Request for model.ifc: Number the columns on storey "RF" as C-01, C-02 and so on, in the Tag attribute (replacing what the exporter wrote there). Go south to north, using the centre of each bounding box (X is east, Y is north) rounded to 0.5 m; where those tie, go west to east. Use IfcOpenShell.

First a look at what the model holds.

```python
import ifcopenshell
import ifcopenshell.util.element
import ifcopenshell.util.placement

model = ifcopenshell.open("model.ifc")
print(model.schema)
storey = next(s for s in model.by_type("IfcBuildingStorey") if s.Name == "RF")
columns = [e for e in ifcopenshell.util.element.get_decomposition(storey) if e.is_a("IfcColumn")]
for e in sorted(columns, key=lambda e: e.id()):
    origin = ifcopenshell.util.placement.get_local_placement(e.ObjectPlacement)[:3, 3]
    print(e.id(), e.Tag, e.Name, origin.round(2) + 0.0, sep=" | ")
```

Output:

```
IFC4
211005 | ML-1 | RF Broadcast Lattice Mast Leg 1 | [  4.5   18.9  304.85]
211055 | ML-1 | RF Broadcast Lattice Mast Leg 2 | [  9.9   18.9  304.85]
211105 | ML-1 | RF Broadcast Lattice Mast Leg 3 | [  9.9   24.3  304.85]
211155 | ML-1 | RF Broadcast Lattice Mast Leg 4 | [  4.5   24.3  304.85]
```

```python
import ifcopenshell
import ifcopenshell.geom
import ifcopenshell.util.element
import ifcopenshell.util.shape

model = ifcopenshell.open("model.ifc")
settings = ifcopenshell.geom.settings()
settings.set("use-world-coords", True)


def centre(element):
    shape = ifcopenshell.geom.create_shape(settings, element)
    return ifcopenshell.util.shape.get_bbox_centroid(shape.geometry)


storey = next(s for s in model.by_type("IfcBuildingStorey") if s.Name == "RF")
columns = [e for e in ifcopenshell.util.element.get_decomposition(storey) if e.is_a("IfcColumn")]

# Insertion points can sit at a corner or the storey origin, so sort by the geometry (in metres).
centres = {e: centre(e) for e in columns}
columns.sort(key=lambda e: (round(centres[e][1] / 0.5), centres[e][0]))

for i, e in enumerate(columns, start=1):
    number = f"C-{i:02d}"
    e.Tag = number
    print(e.id(), number)

model.write("model_rev.ifc")
```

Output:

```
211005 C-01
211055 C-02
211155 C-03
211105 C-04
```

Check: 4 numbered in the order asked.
